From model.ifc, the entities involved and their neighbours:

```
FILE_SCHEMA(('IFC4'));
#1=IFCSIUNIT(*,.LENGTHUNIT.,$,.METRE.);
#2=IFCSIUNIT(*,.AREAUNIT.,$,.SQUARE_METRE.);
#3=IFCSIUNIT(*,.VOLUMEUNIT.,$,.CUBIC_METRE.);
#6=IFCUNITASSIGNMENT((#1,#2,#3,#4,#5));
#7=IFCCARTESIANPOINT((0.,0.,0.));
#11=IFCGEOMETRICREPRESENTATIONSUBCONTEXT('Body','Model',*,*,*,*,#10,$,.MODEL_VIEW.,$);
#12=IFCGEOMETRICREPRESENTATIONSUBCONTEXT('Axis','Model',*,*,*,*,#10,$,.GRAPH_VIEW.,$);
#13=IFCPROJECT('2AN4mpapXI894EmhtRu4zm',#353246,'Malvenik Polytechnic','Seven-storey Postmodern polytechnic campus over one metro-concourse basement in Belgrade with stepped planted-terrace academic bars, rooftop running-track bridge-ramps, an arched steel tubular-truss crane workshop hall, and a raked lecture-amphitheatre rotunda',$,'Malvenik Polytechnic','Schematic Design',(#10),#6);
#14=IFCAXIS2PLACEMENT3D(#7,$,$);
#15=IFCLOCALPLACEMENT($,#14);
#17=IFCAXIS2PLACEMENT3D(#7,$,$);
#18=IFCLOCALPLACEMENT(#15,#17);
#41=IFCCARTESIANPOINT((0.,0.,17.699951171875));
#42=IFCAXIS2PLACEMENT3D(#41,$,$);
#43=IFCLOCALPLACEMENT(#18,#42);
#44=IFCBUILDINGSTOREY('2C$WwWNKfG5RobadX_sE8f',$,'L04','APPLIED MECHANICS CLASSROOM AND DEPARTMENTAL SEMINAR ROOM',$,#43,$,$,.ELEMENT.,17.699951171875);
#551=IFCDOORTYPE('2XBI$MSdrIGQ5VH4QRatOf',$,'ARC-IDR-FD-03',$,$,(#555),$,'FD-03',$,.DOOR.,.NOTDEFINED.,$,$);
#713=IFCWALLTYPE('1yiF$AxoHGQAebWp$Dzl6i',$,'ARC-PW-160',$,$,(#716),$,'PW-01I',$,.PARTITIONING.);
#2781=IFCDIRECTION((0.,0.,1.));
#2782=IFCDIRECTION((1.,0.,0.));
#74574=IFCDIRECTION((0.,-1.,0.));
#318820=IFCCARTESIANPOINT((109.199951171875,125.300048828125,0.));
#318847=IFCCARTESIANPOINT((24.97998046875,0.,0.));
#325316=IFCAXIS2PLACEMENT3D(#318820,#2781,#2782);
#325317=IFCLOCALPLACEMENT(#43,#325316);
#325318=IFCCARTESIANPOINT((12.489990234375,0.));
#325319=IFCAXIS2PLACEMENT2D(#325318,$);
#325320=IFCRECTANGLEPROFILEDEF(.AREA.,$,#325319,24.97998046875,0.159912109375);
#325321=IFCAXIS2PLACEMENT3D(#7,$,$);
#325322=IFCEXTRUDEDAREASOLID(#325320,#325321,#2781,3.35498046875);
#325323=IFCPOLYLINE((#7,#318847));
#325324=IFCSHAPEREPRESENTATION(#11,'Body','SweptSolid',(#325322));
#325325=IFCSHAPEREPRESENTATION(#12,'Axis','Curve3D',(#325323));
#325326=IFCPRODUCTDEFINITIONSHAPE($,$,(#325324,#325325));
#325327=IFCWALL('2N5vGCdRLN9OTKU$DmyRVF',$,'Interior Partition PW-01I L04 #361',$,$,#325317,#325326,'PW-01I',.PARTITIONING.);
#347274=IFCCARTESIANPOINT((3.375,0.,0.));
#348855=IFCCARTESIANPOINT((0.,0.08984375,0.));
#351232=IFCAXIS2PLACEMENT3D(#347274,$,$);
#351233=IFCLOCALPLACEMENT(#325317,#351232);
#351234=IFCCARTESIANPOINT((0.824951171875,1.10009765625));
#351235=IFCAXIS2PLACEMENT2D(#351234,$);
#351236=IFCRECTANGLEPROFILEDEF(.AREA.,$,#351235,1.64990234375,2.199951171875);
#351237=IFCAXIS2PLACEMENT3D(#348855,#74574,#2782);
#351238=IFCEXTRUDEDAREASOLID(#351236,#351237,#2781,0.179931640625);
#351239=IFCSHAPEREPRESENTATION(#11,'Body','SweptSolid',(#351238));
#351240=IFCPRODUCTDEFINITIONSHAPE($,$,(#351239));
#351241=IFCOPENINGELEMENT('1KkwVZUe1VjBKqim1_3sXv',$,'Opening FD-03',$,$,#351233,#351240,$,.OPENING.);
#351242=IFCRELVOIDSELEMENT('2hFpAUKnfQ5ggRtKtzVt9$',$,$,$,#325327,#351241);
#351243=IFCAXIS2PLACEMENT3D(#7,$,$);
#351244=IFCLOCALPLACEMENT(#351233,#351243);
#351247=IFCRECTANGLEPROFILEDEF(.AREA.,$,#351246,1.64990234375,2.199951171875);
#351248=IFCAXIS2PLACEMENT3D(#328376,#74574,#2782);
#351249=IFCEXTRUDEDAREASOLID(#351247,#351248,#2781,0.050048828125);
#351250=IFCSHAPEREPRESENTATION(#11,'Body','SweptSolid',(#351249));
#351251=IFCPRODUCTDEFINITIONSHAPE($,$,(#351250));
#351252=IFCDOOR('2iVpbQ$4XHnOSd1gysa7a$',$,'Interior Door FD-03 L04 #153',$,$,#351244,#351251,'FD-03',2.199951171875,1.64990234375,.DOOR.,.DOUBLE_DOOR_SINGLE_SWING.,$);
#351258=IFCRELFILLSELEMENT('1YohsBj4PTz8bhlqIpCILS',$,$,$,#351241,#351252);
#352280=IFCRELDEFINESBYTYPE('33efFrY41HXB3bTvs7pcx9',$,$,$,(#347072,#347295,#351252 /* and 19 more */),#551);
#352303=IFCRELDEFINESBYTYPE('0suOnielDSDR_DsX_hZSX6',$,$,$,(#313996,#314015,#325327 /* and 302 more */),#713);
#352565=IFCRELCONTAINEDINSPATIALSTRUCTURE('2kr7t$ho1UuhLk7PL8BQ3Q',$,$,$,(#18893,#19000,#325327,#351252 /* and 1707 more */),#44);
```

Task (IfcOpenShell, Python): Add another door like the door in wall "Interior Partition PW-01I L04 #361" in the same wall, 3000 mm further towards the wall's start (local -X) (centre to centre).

```python
import ifcopenshell
import ifcopenshell.api.feature
import ifcopenshell.api.geometry
import ifcopenshell.api.root
import ifcopenshell.geom
import ifcopenshell.util.element
import ifcopenshell.util.placement
import ifcopenshell.util.shape
import ifcopenshell.util.unit

model = ifcopenshell.open("model.ifc")
unit_scale = ifcopenshell.util.unit.calculate_unit_scale(model)
settings = ifcopenshell.geom.settings()


def volume(element):
    """Net volume in cubic metres, openings subtracted."""
    shape = ifcopenshell.geom.create_shape(settings, element)
    return ifcopenshell.util.shape.get_volume(shape.geometry)


door = model.by_guid("2iVpbQ$4XHnOSd1gysa7a$")
opening = door.FillsVoids[0].RelatingOpeningElement
wall = opening.VoidsElements[0].RelatingBuildingElement
before = volume(wall)
shift = ifcopenshell.util.placement.get_local_placement(wall.ObjectPlacement)[:3, 0] * -3 / unit_scale

# copy_class copies the void relationship, type, container and properties, but no geometry.
new_opening = ifcopenshell.api.root.copy_class(model, product=opening)
new_opening.Representation = ifcopenshell.util.element.copy_deep(
    model, opening.Representation, exclude=["IfcGeometricRepresentationContext", "IfcRepresentationMap"]
)
new_door = ifcopenshell.api.root.copy_class(model, product=door)
new_door.Representation = ifcopenshell.util.element.copy_deep(
    model, door.Representation, exclude=["IfcGeometricRepresentationContext", "IfcRepresentationMap"]
)
new_door.Tag = None
ifcopenshell.api.feature.add_filling(model, opening=new_opening, element=new_door)

for old, new in ((opening, new_opening), (door, new_door)):
    matrix = ifcopenshell.util.placement.get_local_placement(old.ObjectPlacement)
    matrix[:3, 3] += shift
    ifcopenshell.api.geometry.edit_object_placement(model, product=new, matrix=matrix, is_si=False)

after = volume(wall)

print(f"wall volume {before:.3f} -> {after:.3f} m3")

model.write("model_v2.ifc")
```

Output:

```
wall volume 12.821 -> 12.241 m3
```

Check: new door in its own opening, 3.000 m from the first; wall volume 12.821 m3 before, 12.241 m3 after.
